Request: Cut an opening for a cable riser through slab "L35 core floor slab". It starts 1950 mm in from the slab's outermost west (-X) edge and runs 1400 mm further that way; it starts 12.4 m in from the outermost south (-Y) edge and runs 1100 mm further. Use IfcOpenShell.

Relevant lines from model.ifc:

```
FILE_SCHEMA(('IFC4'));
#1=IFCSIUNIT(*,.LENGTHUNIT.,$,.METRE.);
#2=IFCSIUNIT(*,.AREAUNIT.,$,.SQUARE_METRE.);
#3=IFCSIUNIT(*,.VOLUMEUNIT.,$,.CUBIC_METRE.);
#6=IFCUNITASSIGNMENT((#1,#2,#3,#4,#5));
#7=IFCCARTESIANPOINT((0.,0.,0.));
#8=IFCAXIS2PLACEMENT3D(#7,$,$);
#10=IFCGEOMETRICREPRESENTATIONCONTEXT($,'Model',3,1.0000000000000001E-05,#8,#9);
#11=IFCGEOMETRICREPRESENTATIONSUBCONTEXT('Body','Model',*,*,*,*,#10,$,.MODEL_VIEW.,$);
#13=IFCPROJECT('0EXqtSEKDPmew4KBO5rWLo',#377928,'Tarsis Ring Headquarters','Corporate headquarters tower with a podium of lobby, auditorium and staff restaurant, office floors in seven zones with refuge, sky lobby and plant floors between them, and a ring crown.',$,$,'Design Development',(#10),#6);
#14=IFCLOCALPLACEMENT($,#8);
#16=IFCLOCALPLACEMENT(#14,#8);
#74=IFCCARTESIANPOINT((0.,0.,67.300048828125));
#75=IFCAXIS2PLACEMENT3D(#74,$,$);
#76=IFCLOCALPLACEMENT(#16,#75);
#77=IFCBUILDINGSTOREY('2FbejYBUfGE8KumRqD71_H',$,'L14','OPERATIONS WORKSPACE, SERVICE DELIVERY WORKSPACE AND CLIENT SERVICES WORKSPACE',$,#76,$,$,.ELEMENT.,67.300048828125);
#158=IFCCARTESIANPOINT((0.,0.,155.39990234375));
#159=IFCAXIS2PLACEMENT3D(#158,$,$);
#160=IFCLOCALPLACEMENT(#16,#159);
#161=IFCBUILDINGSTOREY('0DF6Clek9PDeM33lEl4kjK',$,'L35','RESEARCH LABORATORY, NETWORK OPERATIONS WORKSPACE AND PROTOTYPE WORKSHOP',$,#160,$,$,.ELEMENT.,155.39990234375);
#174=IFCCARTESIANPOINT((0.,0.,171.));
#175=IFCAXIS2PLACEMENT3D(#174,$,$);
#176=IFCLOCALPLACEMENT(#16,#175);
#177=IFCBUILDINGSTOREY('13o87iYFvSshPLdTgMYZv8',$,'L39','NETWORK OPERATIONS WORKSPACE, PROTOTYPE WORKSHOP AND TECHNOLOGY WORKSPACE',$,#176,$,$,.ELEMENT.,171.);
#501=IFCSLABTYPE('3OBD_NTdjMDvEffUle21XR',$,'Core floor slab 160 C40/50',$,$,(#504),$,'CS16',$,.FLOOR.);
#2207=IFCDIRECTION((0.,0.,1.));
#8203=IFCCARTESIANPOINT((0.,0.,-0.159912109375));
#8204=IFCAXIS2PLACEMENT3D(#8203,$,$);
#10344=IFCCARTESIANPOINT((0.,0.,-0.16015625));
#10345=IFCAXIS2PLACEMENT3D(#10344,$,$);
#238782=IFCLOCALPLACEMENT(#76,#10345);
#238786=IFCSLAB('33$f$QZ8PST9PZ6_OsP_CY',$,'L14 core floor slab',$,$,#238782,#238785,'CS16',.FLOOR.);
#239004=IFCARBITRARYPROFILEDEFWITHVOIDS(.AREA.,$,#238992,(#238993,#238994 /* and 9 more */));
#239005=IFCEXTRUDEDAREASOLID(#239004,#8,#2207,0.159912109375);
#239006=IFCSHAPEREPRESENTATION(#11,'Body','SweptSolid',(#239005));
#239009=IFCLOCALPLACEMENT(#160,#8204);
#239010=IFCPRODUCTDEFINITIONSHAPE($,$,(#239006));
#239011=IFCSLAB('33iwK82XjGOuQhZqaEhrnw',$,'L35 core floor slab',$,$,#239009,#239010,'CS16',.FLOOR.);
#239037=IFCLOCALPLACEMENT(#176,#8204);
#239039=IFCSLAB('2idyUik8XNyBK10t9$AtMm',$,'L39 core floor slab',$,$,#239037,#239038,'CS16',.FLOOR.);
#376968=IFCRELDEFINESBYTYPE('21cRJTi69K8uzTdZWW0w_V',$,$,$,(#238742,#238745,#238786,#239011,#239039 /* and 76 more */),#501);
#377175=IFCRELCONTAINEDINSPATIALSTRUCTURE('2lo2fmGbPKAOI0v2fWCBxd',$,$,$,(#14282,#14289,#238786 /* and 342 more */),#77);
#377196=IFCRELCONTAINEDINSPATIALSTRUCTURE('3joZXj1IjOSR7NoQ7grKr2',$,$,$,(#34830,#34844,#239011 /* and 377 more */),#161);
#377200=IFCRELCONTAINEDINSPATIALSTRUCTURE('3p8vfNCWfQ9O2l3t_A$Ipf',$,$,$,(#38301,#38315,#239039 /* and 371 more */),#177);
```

```python
import numpy as np
import ifcopenshell
import ifcopenshell.api.feature
import ifcopenshell.api.geometry
import ifcopenshell.api.root
import ifcopenshell.geom
import ifcopenshell.util.placement
import ifcopenshell.util.representation
import ifcopenshell.util.shape
import ifcopenshell.util.unit

model = ifcopenshell.open("model.ifc")
unit_scale = ifcopenshell.util.unit.calculate_unit_scale(model)
settings = ifcopenshell.geom.settings()


def volume(element):
    """Net volume in cubic metres, openings subtracted."""
    shape = ifcopenshell.geom.create_shape(settings, element)
    return ifcopenshell.util.shape.get_volume(shape.geometry)


slab = model.by_guid("33iwK82XjGOuQhZqaEhrnw")
before = volume(slab)

# Extent in the slab's own axes, in metres. The edges named are its -X and -Y sides.
slab_shape = ifcopenshell.geom.create_shape(settings, slab)
vertices = ifcopenshell.util.shape.get_vertices(slab_shape.geometry)
x_min, y_min, bottom = vertices.min(axis=0)
top = vertices[:, 2].max()

opening = ifcopenshell.api.root.create_entity(model, ifc_class="IfcOpeningElement", name="Cable riser opening", predefined_type="OPENING")
context = ifcopenshell.util.representation.get_context(model, "Model", "Body", "MODEL_VIEW")
width, depth = 1.4, 1.1
outline = [(0.0, 0.0), (width, 0.0), (width, depth), (0.0, depth), (0.0, 0.0)]
# Overshoot both faces by 50 mm so the cut is clean.
shape = ifcopenshell.api.geometry.add_slab_representation(
    model, context=context, depth=top - bottom + 0.1, polyline=outline
)
ifcopenshell.api.geometry.assign_representation(model, product=opening, representation=shape)

matrix = ifcopenshell.util.placement.get_local_placement(slab.ObjectPlacement)
matrix[:, 3] = matrix @ np.append(np.array([x_min + 1.95, y_min + 12.4, bottom - 0.05]) / unit_scale, 1.0)
ifcopenshell.api.geometry.edit_object_placement(model, product=opening, matrix=matrix, is_si=False)
ifcopenshell.api.feature.add_feature(model, feature=opening, element=slab)

after = volume(slab)

print(f"slab volume {before:.3f} -> {after:.3f} m3")

model.write("model_v2.ifc")
```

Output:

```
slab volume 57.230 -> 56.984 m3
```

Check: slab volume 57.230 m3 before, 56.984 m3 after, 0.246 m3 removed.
